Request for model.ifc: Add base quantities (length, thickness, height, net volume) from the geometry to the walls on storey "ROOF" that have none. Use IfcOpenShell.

First a look at what the model holds.

```python
import ifcopenshell
import ifcopenshell.util.element
import ifcopenshell.util.unit

model = ifcopenshell.open("model.ifc")
print(model.schema)
for unit_type in ("LENGTHUNIT", "AREAUNIT", "VOLUMEUNIT"):
    print(unit_type, ifcopenshell.util.unit.calculate_unit_scale(model, unit_type))
storey = next(s for s in model.by_type("IfcBuildingStorey") if s.Name == "ROOF")
walls = [e for e in ifcopenshell.util.element.get_decomposition(storey) if e.is_a("IfcWall")]
for e in sorted(walls, key=lambda e: e.id()):
    print(e.id(), e.is_a(), e.Name, list(ifcopenshell.util.element.get_psets(e, qtos_only=True)), sep=" | ")
```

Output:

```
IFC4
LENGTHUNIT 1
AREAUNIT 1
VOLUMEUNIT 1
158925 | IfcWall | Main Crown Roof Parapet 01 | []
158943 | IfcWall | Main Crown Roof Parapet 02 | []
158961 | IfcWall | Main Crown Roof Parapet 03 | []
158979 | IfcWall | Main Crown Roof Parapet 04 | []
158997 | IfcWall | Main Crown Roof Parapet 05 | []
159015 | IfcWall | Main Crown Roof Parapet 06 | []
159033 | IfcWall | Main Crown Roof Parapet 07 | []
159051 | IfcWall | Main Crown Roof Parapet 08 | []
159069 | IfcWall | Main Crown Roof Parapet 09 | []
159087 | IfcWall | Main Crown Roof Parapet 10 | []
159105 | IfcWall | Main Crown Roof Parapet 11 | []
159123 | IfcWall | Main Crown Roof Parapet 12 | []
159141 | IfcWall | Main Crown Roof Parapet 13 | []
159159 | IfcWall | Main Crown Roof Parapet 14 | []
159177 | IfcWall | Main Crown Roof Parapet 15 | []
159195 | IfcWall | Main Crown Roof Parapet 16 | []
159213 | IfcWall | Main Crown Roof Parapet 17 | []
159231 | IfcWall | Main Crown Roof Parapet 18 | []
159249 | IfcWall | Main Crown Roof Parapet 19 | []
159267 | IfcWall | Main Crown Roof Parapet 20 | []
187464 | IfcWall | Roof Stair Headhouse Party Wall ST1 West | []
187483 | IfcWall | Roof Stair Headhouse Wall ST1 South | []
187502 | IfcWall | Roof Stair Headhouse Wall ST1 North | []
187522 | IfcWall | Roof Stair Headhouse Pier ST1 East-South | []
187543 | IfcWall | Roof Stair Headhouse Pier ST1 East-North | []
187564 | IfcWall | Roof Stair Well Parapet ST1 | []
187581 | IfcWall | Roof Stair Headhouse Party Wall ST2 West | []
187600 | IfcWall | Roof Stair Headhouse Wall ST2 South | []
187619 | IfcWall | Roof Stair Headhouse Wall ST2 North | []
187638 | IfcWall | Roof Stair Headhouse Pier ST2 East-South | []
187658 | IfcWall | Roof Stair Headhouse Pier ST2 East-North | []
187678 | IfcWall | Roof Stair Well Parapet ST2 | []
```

```python
import ifcopenshell
import ifcopenshell.api.pset
import ifcopenshell.geom
import ifcopenshell.util.element
import ifcopenshell.util.shape
import ifcopenshell.util.unit

model = ifcopenshell.open("model.ifc")
unit_scale = ifcopenshell.util.unit.calculate_unit_scale(model)
volume_scale = ifcopenshell.util.unit.calculate_unit_scale(model, "VOLUMEUNIT")
settings = ifcopenshell.geom.settings()

storey = next(s for s in model.by_type("IfcBuildingStorey") if s.Name == "ROOF")
walls = [e for e in ifcopenshell.util.element.get_decomposition(storey) if e.is_a("IfcWall")]

for e in sorted(walls, key=lambda e: e.id()):
    if ifcopenshell.util.element.get_psets(e, qtos_only=True, should_inherit=False):
        continue
    # Geometry comes back in metres, in the element's own axes.
    shape = ifcopenshell.geom.create_shape(settings, e)
    values = {
        "Length": ifcopenshell.util.shape.get_x(shape.geometry) / unit_scale,
        "Width": ifcopenshell.util.shape.get_y(shape.geometry) / unit_scale,
        "Height": ifcopenshell.util.shape.get_z(shape.geometry) / unit_scale,
        "NetVolume": ifcopenshell.util.shape.get_volume(shape.geometry) / volume_scale,
    }
    qto = ifcopenshell.api.pset.add_qto(model, product=e, name="Qto_WallBaseQuantities")
    ifcopenshell.api.pset.edit_qto(model, qto=qto, properties=values)
    print(e.id(), {k: round(v, 3) for k, v in values.items()})

model.write("model_updated.ifc")
```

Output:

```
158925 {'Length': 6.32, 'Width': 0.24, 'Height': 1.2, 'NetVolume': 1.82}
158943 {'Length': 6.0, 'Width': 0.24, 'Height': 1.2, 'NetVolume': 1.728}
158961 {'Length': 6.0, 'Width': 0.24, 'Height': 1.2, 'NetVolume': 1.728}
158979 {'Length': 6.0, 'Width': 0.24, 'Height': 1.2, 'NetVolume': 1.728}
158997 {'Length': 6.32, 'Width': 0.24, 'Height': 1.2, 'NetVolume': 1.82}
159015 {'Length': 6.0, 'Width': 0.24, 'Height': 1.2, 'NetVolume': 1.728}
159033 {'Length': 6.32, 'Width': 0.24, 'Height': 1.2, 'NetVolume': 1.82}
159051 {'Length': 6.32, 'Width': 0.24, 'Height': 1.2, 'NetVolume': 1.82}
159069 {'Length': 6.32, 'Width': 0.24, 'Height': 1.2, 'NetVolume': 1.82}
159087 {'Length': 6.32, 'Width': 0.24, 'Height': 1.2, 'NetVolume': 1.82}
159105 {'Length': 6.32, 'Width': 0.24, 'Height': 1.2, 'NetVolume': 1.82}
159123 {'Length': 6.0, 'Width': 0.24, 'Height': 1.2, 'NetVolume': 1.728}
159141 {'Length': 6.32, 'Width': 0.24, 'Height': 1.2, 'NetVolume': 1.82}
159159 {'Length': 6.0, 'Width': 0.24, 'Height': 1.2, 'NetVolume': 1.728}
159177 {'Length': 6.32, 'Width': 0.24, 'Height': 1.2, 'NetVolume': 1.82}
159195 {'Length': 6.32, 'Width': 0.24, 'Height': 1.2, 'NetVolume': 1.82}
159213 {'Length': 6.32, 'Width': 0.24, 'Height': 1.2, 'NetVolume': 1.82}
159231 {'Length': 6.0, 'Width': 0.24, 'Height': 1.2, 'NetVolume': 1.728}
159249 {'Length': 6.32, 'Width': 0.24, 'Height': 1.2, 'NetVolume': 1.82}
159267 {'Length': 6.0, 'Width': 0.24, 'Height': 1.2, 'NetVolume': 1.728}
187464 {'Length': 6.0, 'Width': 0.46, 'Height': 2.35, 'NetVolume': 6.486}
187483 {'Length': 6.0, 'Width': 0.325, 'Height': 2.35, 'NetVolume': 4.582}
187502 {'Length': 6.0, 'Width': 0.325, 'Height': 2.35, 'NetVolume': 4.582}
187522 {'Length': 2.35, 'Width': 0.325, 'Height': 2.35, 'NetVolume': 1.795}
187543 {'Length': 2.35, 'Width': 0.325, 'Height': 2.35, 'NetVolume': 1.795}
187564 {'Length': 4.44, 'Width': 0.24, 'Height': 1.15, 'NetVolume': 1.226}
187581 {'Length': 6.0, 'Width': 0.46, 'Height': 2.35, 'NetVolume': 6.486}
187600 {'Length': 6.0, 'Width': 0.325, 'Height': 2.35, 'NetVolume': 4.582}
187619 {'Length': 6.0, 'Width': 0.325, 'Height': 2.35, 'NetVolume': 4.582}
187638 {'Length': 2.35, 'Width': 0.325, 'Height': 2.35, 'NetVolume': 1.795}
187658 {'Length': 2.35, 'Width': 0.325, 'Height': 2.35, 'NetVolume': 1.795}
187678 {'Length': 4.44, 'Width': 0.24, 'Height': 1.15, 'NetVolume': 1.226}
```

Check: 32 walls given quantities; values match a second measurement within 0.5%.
